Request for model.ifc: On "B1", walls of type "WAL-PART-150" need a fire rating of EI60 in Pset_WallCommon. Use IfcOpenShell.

First a look at what the model holds.

```python
import ifcopenshell
import ifcopenshell.util.element

model = ifcopenshell.open("model.ifc")
print(model.schema)
storey = next(s for s in model.by_type("IfcBuildingStorey") if s.Name == "B1")
walls = [e for e in ifcopenshell.util.element.get_decomposition(storey) if e.is_a("IfcWall")]
seen = {}
for e in walls:
    element_type = ifcopenshell.util.element.get_type(e)
    key = (element_type.Name if element_type != e and element_type else None, ifcopenshell.util.element.get_pset(e, "Pset_WallCommon", "FireRating"))
    seen[key] = seen.get(key, 0) + 1
for (name, value), count in sorted(seen.items(), key=str):
    print(count, "x", name, "|", value)
```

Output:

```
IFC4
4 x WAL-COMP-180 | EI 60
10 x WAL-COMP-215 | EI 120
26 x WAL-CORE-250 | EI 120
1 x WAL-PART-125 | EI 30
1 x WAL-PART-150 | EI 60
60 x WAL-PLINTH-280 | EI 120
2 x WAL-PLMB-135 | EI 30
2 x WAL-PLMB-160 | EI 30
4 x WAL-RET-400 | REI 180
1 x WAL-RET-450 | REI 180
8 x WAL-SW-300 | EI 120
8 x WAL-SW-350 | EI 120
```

```python
import ifcopenshell
import ifcopenshell.api.pset
import ifcopenshell.util.element

model = ifcopenshell.open("model.ifc")

storey = next(s for s in model.by_type("IfcBuildingStorey") if s.Name == "B1")
walls = [e for e in ifcopenshell.util.element.get_decomposition(storey) if e.is_a("IfcWall")]

count = 0
for e in walls:
    element_type = ifcopenshell.util.element.get_type(e)
    if element_type in (None, e) or element_type.Name != "WAL-PART-150":
        continue
    # add_pset returns the element's existing set when there is one.
    pset = ifcopenshell.api.pset.add_pset(model, product=e, name="Pset_WallCommon")
    ifcopenshell.api.pset.edit_pset(model, pset=pset, properties={"FireRating": "EI60"})
    count += 1

print(count, "walls updated")

model.write("model_edited.ifc")
```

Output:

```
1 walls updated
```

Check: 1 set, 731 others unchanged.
